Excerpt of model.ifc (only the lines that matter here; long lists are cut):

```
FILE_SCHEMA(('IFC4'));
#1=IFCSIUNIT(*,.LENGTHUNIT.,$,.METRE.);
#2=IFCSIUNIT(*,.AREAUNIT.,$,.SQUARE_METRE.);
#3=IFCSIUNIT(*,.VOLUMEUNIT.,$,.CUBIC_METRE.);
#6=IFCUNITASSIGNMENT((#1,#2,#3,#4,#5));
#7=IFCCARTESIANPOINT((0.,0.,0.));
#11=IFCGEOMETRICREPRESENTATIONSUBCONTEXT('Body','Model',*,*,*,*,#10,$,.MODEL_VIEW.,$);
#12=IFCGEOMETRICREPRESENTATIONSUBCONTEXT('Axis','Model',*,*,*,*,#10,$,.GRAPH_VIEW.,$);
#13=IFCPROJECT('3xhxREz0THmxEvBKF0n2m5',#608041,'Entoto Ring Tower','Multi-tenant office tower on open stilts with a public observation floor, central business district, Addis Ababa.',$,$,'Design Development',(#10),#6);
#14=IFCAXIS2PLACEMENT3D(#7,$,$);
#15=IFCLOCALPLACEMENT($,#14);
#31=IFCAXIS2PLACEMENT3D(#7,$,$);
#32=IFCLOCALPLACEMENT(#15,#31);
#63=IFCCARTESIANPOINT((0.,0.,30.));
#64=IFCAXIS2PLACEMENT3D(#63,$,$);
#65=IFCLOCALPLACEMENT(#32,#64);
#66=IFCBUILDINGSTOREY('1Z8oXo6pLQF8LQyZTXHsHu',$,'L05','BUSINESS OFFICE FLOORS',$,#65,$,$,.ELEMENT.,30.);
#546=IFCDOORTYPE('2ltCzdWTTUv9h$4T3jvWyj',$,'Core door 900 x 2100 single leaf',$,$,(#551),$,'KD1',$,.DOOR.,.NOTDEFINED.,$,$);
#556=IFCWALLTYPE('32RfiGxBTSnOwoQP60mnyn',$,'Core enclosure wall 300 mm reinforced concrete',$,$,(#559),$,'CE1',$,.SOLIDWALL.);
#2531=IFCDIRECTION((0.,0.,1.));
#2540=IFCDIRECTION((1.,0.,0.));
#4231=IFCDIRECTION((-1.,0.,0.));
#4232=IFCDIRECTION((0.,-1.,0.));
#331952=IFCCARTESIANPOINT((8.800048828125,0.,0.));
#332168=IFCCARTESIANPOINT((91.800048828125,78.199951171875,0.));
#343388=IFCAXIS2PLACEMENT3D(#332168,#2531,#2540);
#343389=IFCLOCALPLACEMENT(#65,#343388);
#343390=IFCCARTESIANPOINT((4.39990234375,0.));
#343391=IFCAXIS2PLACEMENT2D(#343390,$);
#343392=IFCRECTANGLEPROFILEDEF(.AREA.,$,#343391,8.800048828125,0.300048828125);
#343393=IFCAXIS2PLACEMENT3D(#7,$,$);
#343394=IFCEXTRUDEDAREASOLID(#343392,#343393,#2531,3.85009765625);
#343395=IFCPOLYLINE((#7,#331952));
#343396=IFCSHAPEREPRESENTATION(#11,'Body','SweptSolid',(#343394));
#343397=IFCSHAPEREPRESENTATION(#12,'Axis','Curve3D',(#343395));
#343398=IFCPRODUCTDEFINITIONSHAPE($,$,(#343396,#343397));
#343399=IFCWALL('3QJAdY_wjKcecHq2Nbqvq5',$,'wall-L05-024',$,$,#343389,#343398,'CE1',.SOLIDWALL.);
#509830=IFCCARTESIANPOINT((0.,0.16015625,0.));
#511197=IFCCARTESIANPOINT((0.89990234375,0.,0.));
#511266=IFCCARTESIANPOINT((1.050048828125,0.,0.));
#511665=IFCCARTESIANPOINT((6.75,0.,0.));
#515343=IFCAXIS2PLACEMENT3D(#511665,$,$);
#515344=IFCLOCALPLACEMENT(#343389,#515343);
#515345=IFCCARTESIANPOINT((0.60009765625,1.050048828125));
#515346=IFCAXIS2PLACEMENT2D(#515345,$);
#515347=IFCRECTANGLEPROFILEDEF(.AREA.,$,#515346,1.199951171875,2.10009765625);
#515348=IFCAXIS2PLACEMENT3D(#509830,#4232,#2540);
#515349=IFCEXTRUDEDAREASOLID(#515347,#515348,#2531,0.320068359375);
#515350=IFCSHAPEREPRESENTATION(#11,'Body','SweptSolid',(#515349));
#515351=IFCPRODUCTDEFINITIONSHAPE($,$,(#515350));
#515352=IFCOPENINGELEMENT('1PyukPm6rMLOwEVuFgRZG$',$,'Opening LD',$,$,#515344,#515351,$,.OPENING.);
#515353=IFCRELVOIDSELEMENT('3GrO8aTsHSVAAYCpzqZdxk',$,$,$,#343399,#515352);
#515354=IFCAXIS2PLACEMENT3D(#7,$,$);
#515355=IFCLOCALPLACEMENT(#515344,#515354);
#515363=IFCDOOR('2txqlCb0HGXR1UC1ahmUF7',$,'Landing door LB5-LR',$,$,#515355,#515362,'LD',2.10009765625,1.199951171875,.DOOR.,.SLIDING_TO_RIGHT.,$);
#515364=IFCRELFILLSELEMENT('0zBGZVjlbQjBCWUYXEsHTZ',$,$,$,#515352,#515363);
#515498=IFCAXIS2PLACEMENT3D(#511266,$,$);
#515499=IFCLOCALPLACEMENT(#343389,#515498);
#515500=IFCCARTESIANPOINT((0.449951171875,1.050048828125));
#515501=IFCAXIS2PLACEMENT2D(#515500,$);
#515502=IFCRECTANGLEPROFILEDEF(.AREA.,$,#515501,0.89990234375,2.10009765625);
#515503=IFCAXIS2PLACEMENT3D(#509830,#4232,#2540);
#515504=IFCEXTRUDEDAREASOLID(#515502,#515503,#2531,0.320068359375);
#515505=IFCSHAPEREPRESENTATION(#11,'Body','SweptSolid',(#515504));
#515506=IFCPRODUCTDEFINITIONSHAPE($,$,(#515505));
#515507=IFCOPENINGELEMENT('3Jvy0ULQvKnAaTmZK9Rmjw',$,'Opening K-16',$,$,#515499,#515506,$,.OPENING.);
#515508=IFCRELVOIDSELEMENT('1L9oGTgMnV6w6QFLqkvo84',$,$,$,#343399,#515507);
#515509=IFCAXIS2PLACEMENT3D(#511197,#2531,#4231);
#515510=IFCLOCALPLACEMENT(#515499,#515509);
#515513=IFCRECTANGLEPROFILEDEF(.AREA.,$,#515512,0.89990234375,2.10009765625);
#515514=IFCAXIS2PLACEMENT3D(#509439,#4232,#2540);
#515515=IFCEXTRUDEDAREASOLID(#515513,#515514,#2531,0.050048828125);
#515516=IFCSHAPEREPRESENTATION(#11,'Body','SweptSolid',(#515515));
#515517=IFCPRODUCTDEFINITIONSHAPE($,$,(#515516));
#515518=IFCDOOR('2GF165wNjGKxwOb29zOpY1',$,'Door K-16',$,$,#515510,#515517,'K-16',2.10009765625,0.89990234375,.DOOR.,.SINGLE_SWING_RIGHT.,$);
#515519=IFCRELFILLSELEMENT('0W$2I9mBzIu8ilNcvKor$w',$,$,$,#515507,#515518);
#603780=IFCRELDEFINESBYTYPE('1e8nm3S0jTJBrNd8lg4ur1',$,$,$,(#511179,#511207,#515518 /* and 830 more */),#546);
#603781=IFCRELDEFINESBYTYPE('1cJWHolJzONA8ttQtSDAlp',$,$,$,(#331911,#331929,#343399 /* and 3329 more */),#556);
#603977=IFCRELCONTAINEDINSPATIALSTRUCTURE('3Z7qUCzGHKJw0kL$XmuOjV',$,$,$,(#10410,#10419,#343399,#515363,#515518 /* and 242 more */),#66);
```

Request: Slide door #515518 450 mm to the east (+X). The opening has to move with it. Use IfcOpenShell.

```python
import ifcopenshell
import ifcopenshell.api.geometry
import ifcopenshell.util.placement

model = ifcopenshell.open("model.ifc")

door = model.by_guid("2GF165wNjGKxwOb29zOpY1")
opening = door.FillsVoids[0].RelatingOpeningElement
wall = opening.VoidsElements[0].RelatingBuildingElement

wall_matrix = ifcopenshell.util.placement.get_local_placement(wall.ObjectPlacement)
shift = wall_matrix[:3, 0] * 0.45
before = ifcopenshell.util.placement.get_local_placement(door.ObjectPlacement)[:3, 3].copy()

# The door is placed relative to its opening, so it follows when the opening moves.
matrix = ifcopenshell.util.placement.get_local_placement(opening.ObjectPlacement)
matrix[:3, 3] += shift
ifcopenshell.api.geometry.edit_object_placement(
    model, product=opening, matrix=matrix, is_si=False, should_transform_children=True
)

after = ifcopenshell.util.placement.get_local_placement(door.ObjectPlacement)[:3, 3]
print("door moved by", (after - before).round(3) + 0.0)

model.write("model_rev.ifc")
```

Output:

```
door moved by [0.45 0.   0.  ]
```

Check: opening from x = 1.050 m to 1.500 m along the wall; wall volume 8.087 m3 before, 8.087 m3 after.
